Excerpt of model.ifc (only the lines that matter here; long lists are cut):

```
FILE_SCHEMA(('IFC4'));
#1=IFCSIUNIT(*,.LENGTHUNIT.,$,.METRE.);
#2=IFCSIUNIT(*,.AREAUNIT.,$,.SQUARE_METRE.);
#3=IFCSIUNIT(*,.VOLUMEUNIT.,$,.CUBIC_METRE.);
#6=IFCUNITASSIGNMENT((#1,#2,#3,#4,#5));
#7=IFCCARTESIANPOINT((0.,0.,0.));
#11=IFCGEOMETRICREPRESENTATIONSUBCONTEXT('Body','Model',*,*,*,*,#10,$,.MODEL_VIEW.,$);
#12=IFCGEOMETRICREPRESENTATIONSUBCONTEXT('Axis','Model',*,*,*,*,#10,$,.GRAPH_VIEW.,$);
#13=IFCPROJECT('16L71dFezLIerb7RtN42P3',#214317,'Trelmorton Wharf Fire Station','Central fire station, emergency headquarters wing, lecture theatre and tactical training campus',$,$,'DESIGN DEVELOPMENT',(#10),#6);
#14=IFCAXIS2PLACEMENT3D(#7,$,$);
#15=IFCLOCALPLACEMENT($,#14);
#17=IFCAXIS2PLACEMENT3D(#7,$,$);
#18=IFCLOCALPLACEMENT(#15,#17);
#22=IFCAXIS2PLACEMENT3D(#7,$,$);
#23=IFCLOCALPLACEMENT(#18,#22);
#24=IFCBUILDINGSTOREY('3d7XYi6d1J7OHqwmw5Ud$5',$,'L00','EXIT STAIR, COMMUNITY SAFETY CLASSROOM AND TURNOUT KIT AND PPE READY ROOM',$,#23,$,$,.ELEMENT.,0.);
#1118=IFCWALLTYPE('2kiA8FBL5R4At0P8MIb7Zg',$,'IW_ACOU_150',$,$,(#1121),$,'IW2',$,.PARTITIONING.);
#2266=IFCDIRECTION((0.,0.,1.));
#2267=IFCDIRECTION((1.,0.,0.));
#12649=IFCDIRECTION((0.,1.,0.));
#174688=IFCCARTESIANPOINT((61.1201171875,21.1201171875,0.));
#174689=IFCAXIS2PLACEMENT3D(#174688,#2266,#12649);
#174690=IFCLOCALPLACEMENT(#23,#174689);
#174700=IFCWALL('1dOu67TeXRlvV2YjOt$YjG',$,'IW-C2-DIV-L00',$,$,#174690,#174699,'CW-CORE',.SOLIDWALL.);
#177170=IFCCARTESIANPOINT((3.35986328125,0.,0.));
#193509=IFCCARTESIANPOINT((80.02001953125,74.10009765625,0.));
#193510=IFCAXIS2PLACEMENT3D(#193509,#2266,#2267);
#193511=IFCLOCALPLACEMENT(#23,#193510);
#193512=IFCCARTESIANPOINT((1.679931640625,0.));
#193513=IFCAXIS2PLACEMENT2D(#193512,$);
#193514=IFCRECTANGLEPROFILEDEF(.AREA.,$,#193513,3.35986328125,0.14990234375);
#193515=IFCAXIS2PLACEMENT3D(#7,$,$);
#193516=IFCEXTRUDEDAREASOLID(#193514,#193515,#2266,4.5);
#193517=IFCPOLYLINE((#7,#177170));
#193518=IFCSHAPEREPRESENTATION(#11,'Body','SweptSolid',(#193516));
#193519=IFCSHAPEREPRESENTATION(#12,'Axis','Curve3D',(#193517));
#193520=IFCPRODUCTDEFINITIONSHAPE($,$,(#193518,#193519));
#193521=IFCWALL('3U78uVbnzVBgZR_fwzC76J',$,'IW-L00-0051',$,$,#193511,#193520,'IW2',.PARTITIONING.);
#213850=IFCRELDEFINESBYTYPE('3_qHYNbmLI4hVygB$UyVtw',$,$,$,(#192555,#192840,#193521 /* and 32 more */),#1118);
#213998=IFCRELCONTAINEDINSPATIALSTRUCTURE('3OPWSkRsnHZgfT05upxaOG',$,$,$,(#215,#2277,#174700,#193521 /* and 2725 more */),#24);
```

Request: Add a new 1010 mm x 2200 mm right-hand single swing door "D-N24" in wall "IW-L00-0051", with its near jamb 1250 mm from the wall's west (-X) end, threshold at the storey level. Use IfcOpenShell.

```python
import numpy as np
import ifcopenshell
import ifcopenshell.api.feature
import ifcopenshell.api.geometry
import ifcopenshell.api.root
import ifcopenshell.api.spatial
import ifcopenshell.geom
import ifcopenshell.util.element
import ifcopenshell.util.placement
import ifcopenshell.util.representation
import ifcopenshell.util.shape
import ifcopenshell.util.unit

model = ifcopenshell.open("model.ifc")
unit_scale = ifcopenshell.util.unit.calculate_unit_scale(model)
settings = ifcopenshell.geom.settings()


def volume(element):
    """Net volume in cubic metres, openings subtracted."""
    shape = ifcopenshell.geom.create_shape(settings, element)
    return ifcopenshell.util.shape.get_volume(shape.geometry)


wall = model.by_id(193521)
storey = ifcopenshell.util.element.get_container(wall, ifc_class="IfcBuildingStorey")
context = ifcopenshell.util.representation.get_context(model, "Model", "Body", "MODEL_VIEW")
before = volume(wall)

width, height, from_end, sill = 1.01, 2.2, 1.25, 0.0  # metres

# The wall runs along its own X axis, and the end named is its -X end.
wall_shape = ifcopenshell.geom.create_shape(settings, wall)
x, y, z = ifcopenshell.util.shape.get_vertices(wall_shape.geometry).T
start = x.min() + from_end
face, thickness = float(y.min()), float(y.max() - y.min())
wall_matrix = ifcopenshell.util.placement.get_local_placement(wall.ObjectPlacement)
level = ifcopenshell.util.placement.get_local_placement(storey.ObjectPlacement)[2, 3]


def in_wall(x, y):
    """Placement at x, y metres in the wall's axes, at sill height."""
    matrix = wall_matrix.copy()
    matrix[:, 3] = wall_matrix @ np.array([x / unit_scale, y / unit_scale, 0.0, 1.0])
    matrix[2, 3] = level + sill / unit_scale
    return matrix


# Opening: a box that overshoots both wall faces by 50 mm.
opening = ifcopenshell.api.root.create_entity(model, ifc_class="IfcOpeningElement", predefined_type="OPENING")
box = ifcopenshell.api.geometry.add_wall_representation(
    model, context=context, length=width, height=height, thickness=thickness + 0.1
)
ifcopenshell.api.geometry.assign_representation(model, product=opening, representation=box)
ifcopenshell.api.geometry.edit_object_placement(model, product=opening, matrix=in_wall(start, face - 0.05), is_si=False)
ifcopenshell.api.feature.add_feature(model, feature=opening, element=wall)

door = ifcopenshell.api.root.create_entity(model, ifc_class="IfcDoor", name="D-N24", predefined_type="DOOR")
door.OverallWidth, door.OverallHeight = width / unit_scale, height / unit_scale
door.OperationType = "SINGLE_SWING_RIGHT"
body = ifcopenshell.api.geometry.add_door_representation(
    model,
    context=context,
    overall_width=door.OverallWidth,
    overall_height=door.OverallHeight,
    operation_type="SINGLE_SWING_RIGHT",
    lining_properties={"LiningDepth": thickness / unit_scale, "ThresholdDepth": thickness / unit_scale},
)
ifcopenshell.api.geometry.assign_representation(model, product=door, representation=body)
ifcopenshell.api.spatial.assign_container(model, products=[door], relating_structure=storey)
ifcopenshell.api.feature.add_filling(model, opening=opening, element=door)

# The lining spans the wall, so the door starts at the wall face.
ifcopenshell.api.geometry.edit_object_placement(model, product=door, matrix=in_wall(start, face), is_si=False)

after = volume(wall)

print(f"wall volume {before:.3f} -> {after:.3f} m3")

model.write("model_updated.ifc")
```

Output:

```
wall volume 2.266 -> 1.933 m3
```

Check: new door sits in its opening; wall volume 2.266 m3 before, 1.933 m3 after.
